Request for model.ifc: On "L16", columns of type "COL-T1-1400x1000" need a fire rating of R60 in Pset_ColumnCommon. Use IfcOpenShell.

First a look at what the model holds.

```python
import ifcopenshell
import ifcopenshell.util.element

model = ifcopenshell.open("model.ifc")
print(model.schema)
storey = next(s for s in model.by_type("IfcBuildingStorey") if s.Name == "L16")
columns = [e for e in ifcopenshell.util.element.get_decomposition(storey) if e.is_a("IfcColumn")]
seen = {}
for e in columns:
    element_type = ifcopenshell.util.element.get_type(e)
    key = (element_type.Name if element_type != e and element_type else None, ifcopenshell.util.element.get_pset(e, "Pset_ColumnCommon", "FireRating"))
    seen[key] = seen.get(key, 0) + 1
for (name, value), count in sorted(seen.items(), key=str):
    print(count, "x", name, "|", value)
```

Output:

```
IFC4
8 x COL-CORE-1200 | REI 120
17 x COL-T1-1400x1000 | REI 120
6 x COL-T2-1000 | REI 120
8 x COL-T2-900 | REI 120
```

```python
import ifcopenshell
import ifcopenshell.api.pset
import ifcopenshell.util.element

model = ifcopenshell.open("model.ifc")

storey = next(s for s in model.by_type("IfcBuildingStorey") if s.Name == "L16")
columns = [e for e in ifcopenshell.util.element.get_decomposition(storey) if e.is_a("IfcColumn")]

count = 0
for e in columns:
    element_type = ifcopenshell.util.element.get_type(e)
    if element_type in (None, e) or element_type.Name != "COL-T1-1400x1000":
        continue
    # add_pset returns the element's existing set when there is one.
    pset = ifcopenshell.api.pset.add_pset(model, product=e, name="Pset_ColumnCommon")
    ifcopenshell.api.pset.edit_pset(model, pset=pset, properties={"FireRating": "R60"})
    count += 1

print(count, "columns updated")

model.write("model-out.ifc")
```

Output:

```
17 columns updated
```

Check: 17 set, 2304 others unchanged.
